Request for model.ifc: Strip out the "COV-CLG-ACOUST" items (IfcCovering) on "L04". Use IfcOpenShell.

First a look at what the model holds.

```python
import ifcopenshell
import ifcopenshell.util.element

model = ifcopenshell.open("model.ifc")
print(model.schema)
storey = next(s for s in model.by_type("IfcBuildingStorey") if s.Name == "L04")
coverings = [e for e in ifcopenshell.util.element.get_decomposition(storey) if e.is_a("IfcCovering")]
seen = {}
for e in coverings:
    element_type = ifcopenshell.util.element.get_type(e)
    name = element_type.Name if element_type not in (None, e) else None
    seen[name] = seen.get(name, 0) + 1
for name, count in sorted(seen.items(), key=str):
    print(count, "x", name)
```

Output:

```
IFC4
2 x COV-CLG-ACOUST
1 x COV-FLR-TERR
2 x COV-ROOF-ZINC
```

```python
import ifcopenshell
import ifcopenshell.api.root
import ifcopenshell.util.element

model = ifcopenshell.open("model.ifc")

storey = next(s for s in model.by_type("IfcBuildingStorey") if s.Name == "L04")
coverings = [e for e in ifcopenshell.util.element.get_decomposition(storey) if e.is_a("IfcCovering")]
targets = [e for e in coverings if (t := ifcopenshell.util.element.get_type(e)) not in (None, e) and t.Name == "COV-CLG-ACOUST"]

for e in targets:
    ifcopenshell.api.root.remove_product(model, product=e)
print(len(targets), "removed")

model.write("model-out.ifc")
```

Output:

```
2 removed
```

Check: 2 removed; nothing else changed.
